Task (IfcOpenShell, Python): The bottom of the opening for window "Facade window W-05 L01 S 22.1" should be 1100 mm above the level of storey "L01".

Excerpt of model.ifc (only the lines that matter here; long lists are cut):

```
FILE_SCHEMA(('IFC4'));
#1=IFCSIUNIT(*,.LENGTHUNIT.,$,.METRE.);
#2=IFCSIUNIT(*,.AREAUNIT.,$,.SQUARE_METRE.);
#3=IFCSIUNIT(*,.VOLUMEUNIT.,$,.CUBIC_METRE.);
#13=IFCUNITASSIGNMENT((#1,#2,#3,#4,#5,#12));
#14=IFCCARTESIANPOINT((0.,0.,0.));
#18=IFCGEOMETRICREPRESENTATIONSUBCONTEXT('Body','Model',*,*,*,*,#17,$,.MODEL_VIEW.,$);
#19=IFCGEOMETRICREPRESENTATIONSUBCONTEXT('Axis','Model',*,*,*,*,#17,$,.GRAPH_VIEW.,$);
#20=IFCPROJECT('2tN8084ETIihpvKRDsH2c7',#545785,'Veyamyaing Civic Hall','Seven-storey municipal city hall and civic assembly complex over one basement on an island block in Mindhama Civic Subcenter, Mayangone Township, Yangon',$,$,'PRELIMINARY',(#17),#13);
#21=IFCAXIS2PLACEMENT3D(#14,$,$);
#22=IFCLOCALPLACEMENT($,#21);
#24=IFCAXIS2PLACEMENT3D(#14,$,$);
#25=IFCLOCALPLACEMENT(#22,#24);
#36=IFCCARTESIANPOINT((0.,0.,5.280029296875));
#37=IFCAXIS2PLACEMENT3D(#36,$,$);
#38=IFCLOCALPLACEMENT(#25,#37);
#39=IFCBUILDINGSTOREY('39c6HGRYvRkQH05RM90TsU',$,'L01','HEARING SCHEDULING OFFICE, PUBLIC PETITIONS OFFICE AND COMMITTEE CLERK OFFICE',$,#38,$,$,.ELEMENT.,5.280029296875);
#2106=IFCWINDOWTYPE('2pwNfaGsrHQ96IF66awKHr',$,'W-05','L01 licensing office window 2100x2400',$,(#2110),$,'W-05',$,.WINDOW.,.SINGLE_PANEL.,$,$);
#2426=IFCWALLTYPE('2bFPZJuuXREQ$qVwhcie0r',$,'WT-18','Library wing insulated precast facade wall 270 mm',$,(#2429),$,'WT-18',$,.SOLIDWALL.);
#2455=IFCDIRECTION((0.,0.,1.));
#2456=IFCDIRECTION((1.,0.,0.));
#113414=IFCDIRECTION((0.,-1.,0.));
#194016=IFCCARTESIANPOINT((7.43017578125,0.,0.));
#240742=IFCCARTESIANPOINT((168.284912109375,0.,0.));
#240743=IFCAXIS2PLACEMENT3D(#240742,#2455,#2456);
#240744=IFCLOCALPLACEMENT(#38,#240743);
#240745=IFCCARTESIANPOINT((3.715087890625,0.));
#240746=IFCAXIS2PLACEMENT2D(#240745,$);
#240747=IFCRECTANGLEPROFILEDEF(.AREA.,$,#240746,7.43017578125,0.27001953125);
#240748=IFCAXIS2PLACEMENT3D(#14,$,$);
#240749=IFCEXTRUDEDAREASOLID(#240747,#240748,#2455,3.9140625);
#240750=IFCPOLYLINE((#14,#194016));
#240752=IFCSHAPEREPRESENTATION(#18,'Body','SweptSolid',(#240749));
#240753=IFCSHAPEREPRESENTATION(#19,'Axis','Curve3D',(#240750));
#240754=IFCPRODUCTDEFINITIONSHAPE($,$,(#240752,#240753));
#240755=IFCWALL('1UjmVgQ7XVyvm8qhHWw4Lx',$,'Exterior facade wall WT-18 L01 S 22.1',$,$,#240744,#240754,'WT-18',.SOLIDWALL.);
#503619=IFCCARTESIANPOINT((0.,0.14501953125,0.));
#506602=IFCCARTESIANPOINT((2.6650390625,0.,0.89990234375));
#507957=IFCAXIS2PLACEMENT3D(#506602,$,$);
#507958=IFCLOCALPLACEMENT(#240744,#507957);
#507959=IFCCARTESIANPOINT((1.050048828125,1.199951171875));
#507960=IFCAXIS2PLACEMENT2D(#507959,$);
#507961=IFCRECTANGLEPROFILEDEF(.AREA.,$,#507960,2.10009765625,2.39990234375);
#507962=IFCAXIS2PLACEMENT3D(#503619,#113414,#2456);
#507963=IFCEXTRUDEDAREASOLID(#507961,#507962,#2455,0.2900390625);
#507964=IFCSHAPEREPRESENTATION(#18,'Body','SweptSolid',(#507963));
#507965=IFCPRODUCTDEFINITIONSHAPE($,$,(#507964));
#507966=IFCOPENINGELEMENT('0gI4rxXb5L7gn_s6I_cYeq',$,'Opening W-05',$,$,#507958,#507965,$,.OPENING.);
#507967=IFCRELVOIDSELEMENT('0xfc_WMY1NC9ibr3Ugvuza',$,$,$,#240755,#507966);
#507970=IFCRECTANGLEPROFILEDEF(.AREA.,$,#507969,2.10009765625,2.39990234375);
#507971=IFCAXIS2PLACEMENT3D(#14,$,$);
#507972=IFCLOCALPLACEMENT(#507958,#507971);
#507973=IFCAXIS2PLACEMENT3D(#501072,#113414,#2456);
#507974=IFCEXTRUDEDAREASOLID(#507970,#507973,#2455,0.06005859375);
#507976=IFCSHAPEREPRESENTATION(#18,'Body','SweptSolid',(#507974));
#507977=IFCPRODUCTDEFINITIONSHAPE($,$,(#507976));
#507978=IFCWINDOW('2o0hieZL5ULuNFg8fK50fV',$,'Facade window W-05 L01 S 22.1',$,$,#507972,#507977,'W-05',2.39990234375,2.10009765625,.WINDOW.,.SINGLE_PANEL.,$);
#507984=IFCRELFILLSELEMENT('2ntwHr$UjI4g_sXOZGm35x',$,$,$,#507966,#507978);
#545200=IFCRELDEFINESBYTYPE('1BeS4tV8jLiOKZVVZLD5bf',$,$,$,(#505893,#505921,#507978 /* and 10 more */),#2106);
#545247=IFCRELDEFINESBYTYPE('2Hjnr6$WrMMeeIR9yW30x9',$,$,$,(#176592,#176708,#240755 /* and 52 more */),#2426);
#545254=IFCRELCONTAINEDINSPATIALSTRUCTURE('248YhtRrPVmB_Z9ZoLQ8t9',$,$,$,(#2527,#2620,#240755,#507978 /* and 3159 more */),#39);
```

```python
import numpy as np
import ifcopenshell
import ifcopenshell.api.geometry
import ifcopenshell.geom
import ifcopenshell.util.element
import ifcopenshell.util.placement
import ifcopenshell.util.shape
import ifcopenshell.util.unit

model = ifcopenshell.open("model.ifc")
unit_scale = ifcopenshell.util.unit.calculate_unit_scale(model)

window = model.by_id(507978)
opening = window.FillsVoids[0].RelatingOpeningElement
storey = ifcopenshell.util.element.get_container(window, ifc_class="IfcBuildingStorey")
level = ifcopenshell.util.placement.get_local_placement(storey.ObjectPlacement)[2, 3]

# The opening's origin need not be at the sill, so measure its lowest point.
shape = ifcopenshell.geom.create_shape(ifcopenshell.geom.settings(), opening)
bottom = ifcopenshell.util.shape.get_shape_bottom_elevation(shape, shape.geometry) / unit_scale
dz = level + 1.1 - bottom

shift = np.array([0.0, 0.0, dz])
# The window is placed relative to its opening, so it follows when the opening moves.
matrix = ifcopenshell.util.placement.get_local_placement(opening.ObjectPlacement)
matrix[:3, 3] += shift
ifcopenshell.api.geometry.edit_object_placement(
    model, product=opening, matrix=matrix, is_si=False, should_transform_children=True
)

print(f"moved by {dz * unit_scale:+.3f} m")

model.write("model_updated.ifc")
```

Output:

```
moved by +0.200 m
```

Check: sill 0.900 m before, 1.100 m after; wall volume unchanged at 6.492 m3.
